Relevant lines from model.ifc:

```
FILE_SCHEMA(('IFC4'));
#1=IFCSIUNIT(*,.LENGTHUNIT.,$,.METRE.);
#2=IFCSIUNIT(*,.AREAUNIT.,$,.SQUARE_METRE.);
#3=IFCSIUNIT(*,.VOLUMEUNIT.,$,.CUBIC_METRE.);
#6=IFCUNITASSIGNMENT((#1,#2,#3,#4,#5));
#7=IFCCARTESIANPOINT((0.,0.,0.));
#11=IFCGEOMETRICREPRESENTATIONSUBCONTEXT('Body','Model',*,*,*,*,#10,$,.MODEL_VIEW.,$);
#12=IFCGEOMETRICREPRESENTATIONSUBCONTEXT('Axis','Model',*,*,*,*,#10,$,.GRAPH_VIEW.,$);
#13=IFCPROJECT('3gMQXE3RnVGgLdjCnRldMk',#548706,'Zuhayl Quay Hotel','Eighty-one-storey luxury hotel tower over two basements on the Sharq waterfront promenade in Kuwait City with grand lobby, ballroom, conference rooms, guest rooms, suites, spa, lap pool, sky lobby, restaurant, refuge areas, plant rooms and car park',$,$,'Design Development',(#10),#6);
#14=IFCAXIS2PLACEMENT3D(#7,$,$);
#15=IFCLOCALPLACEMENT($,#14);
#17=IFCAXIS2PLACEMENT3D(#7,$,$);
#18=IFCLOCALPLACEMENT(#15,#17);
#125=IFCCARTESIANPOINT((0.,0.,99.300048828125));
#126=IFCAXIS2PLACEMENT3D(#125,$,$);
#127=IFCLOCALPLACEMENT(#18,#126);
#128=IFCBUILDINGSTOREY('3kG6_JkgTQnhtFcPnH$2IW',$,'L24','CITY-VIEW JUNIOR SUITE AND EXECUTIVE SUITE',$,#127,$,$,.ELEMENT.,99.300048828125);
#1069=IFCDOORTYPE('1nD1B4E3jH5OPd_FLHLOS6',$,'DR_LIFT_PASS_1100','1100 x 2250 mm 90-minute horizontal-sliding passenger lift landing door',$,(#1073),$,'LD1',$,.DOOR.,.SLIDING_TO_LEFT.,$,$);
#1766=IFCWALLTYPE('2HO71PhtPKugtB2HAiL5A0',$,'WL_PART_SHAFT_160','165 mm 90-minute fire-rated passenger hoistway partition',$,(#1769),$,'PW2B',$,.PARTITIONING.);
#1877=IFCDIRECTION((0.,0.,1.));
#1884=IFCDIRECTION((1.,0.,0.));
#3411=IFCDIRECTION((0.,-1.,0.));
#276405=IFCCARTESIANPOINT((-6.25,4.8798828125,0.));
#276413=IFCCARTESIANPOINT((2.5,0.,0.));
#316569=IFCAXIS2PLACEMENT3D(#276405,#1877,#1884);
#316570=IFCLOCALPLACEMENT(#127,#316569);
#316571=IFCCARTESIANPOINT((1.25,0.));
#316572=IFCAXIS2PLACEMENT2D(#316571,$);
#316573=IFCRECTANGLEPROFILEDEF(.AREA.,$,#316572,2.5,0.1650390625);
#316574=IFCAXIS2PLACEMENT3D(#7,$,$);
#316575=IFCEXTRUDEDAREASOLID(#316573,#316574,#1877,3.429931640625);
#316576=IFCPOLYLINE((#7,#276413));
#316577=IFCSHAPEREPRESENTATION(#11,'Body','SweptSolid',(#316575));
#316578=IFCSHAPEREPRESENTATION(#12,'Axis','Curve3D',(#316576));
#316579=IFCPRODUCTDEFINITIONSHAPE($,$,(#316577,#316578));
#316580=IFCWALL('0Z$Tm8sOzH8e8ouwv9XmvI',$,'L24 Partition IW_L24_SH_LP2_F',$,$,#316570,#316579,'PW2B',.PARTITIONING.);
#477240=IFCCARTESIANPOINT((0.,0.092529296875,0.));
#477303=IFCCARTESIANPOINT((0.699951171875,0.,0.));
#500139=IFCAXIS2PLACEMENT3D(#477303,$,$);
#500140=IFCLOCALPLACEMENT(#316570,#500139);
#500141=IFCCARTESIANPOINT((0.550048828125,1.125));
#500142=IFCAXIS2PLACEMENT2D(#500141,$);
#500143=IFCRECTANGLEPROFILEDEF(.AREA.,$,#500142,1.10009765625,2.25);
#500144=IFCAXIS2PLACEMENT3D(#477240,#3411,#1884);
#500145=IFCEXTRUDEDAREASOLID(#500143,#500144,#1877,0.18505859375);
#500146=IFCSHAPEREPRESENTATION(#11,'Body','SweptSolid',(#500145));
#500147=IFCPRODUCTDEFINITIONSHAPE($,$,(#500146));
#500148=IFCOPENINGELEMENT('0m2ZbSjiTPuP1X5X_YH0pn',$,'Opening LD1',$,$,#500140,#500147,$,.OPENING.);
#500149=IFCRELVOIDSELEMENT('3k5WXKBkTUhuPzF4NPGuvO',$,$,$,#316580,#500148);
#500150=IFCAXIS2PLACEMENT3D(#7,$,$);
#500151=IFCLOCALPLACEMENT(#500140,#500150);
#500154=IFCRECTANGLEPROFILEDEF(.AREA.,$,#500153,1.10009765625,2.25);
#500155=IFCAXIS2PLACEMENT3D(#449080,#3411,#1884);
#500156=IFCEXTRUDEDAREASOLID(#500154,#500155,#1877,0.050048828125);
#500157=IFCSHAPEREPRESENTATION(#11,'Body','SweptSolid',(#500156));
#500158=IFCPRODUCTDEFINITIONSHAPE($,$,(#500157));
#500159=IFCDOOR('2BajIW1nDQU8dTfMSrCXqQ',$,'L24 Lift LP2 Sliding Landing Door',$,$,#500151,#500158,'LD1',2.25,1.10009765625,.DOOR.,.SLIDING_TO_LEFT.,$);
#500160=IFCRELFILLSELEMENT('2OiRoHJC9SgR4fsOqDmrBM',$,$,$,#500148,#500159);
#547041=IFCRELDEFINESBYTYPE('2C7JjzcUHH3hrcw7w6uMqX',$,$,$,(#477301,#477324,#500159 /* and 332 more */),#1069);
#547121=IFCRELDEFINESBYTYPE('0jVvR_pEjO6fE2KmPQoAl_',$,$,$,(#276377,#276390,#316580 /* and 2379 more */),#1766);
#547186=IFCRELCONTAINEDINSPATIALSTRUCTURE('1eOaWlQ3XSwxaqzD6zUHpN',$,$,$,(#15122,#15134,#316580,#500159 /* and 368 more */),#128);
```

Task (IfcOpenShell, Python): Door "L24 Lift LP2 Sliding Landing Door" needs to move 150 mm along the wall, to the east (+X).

```python
import ifcopenshell
import ifcopenshell.api.geometry
import ifcopenshell.util.placement
import ifcopenshell.util.unit

model = ifcopenshell.open("model.ifc")
unit_scale = ifcopenshell.util.unit.calculate_unit_scale(model)

door = model.by_guid("2BajIW1nDQU8dTfMSrCXqQ")
opening = door.FillsVoids[0].RelatingOpeningElement
wall = opening.VoidsElements[0].RelatingBuildingElement

wall_matrix = ifcopenshell.util.placement.get_local_placement(wall.ObjectPlacement)
shift = wall_matrix[:3, 0] * 0.15 / unit_scale
before = ifcopenshell.util.placement.get_local_placement(door.ObjectPlacement)[:3, 3].copy()

# The door is placed relative to its opening, so it follows when the opening moves.
matrix = ifcopenshell.util.placement.get_local_placement(opening.ObjectPlacement)
matrix[:3, 3] += shift
ifcopenshell.api.geometry.edit_object_placement(
    model, product=opening, matrix=matrix, is_si=False, should_transform_children=True
)

after = ifcopenshell.util.placement.get_local_placement(door.ObjectPlacement)[:3, 3]
print("door moved by", (after - before).round(3) + 0.0)

model.write("model_v2.ifc")
```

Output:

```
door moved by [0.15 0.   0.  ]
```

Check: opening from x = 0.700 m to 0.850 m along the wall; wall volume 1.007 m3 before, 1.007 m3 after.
